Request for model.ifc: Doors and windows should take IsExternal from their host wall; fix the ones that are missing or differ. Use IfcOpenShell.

First a look at what the model holds.

```python
import ifcopenshell
import ifcopenshell.util.element

model = ifcopenshell.open("model.ifc")
print(model.schema)
seen = {}
for e in model.by_type("IfcDoor") + model.by_type("IfcWindow"):
    if not e.FillsVoids:
        continue
    host = e.FillsVoids[0].RelatingOpeningElement.VoidsElements[0].RelatingBuildingElement
    own = ifcopenshell.util.element.get_pset(e, f"Pset_{e.is_a()[3:].removesuffix('StandardCase')}Common", "IsExternal")
    wall = ifcopenshell.util.element.get_pset(host, "Pset_WallCommon", "IsExternal")
    seen[e.is_a(), own, wall] = seen.get((e.is_a(), own, wall), 0) + 1
for (cls, own, wall), count in sorted(seen.items(), key=str):
    print(count, cls, "IsExternal:", own, "| host wall:", wall)
```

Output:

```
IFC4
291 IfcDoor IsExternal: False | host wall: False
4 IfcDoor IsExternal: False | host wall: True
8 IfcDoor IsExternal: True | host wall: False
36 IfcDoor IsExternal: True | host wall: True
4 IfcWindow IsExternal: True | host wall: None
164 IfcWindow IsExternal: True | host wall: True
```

```python
import ifcopenshell
import ifcopenshell.api.pset
import ifcopenshell.util.element

model = ifcopenshell.open("model.ifc")

count = 0
for ifc_class, pset_name in (("IfcDoor", "Pset_DoorCommon"), ("IfcWindow", "Pset_WindowCommon")):
    for e in model.by_type(ifc_class):
        if not e.FillsVoids:
            continue
        host = e.FillsVoids[0].RelatingOpeningElement.VoidsElements[0].RelatingBuildingElement
        external = ifcopenshell.util.element.get_pset(host, "Pset_WallCommon", "IsExternal")
        if external is None or ifcopenshell.util.element.get_pset(e, pset_name, "IsExternal") == external:
            continue
        pset = ifcopenshell.api.pset.add_pset(model, product=e, name=pset_name)
        ifcopenshell.api.pset.edit_pset(model, pset=pset, properties={"IsExternal": external})
        count += 1

print(count, "updated")

model.write("model_rev.ifc")
```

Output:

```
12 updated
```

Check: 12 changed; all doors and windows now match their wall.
